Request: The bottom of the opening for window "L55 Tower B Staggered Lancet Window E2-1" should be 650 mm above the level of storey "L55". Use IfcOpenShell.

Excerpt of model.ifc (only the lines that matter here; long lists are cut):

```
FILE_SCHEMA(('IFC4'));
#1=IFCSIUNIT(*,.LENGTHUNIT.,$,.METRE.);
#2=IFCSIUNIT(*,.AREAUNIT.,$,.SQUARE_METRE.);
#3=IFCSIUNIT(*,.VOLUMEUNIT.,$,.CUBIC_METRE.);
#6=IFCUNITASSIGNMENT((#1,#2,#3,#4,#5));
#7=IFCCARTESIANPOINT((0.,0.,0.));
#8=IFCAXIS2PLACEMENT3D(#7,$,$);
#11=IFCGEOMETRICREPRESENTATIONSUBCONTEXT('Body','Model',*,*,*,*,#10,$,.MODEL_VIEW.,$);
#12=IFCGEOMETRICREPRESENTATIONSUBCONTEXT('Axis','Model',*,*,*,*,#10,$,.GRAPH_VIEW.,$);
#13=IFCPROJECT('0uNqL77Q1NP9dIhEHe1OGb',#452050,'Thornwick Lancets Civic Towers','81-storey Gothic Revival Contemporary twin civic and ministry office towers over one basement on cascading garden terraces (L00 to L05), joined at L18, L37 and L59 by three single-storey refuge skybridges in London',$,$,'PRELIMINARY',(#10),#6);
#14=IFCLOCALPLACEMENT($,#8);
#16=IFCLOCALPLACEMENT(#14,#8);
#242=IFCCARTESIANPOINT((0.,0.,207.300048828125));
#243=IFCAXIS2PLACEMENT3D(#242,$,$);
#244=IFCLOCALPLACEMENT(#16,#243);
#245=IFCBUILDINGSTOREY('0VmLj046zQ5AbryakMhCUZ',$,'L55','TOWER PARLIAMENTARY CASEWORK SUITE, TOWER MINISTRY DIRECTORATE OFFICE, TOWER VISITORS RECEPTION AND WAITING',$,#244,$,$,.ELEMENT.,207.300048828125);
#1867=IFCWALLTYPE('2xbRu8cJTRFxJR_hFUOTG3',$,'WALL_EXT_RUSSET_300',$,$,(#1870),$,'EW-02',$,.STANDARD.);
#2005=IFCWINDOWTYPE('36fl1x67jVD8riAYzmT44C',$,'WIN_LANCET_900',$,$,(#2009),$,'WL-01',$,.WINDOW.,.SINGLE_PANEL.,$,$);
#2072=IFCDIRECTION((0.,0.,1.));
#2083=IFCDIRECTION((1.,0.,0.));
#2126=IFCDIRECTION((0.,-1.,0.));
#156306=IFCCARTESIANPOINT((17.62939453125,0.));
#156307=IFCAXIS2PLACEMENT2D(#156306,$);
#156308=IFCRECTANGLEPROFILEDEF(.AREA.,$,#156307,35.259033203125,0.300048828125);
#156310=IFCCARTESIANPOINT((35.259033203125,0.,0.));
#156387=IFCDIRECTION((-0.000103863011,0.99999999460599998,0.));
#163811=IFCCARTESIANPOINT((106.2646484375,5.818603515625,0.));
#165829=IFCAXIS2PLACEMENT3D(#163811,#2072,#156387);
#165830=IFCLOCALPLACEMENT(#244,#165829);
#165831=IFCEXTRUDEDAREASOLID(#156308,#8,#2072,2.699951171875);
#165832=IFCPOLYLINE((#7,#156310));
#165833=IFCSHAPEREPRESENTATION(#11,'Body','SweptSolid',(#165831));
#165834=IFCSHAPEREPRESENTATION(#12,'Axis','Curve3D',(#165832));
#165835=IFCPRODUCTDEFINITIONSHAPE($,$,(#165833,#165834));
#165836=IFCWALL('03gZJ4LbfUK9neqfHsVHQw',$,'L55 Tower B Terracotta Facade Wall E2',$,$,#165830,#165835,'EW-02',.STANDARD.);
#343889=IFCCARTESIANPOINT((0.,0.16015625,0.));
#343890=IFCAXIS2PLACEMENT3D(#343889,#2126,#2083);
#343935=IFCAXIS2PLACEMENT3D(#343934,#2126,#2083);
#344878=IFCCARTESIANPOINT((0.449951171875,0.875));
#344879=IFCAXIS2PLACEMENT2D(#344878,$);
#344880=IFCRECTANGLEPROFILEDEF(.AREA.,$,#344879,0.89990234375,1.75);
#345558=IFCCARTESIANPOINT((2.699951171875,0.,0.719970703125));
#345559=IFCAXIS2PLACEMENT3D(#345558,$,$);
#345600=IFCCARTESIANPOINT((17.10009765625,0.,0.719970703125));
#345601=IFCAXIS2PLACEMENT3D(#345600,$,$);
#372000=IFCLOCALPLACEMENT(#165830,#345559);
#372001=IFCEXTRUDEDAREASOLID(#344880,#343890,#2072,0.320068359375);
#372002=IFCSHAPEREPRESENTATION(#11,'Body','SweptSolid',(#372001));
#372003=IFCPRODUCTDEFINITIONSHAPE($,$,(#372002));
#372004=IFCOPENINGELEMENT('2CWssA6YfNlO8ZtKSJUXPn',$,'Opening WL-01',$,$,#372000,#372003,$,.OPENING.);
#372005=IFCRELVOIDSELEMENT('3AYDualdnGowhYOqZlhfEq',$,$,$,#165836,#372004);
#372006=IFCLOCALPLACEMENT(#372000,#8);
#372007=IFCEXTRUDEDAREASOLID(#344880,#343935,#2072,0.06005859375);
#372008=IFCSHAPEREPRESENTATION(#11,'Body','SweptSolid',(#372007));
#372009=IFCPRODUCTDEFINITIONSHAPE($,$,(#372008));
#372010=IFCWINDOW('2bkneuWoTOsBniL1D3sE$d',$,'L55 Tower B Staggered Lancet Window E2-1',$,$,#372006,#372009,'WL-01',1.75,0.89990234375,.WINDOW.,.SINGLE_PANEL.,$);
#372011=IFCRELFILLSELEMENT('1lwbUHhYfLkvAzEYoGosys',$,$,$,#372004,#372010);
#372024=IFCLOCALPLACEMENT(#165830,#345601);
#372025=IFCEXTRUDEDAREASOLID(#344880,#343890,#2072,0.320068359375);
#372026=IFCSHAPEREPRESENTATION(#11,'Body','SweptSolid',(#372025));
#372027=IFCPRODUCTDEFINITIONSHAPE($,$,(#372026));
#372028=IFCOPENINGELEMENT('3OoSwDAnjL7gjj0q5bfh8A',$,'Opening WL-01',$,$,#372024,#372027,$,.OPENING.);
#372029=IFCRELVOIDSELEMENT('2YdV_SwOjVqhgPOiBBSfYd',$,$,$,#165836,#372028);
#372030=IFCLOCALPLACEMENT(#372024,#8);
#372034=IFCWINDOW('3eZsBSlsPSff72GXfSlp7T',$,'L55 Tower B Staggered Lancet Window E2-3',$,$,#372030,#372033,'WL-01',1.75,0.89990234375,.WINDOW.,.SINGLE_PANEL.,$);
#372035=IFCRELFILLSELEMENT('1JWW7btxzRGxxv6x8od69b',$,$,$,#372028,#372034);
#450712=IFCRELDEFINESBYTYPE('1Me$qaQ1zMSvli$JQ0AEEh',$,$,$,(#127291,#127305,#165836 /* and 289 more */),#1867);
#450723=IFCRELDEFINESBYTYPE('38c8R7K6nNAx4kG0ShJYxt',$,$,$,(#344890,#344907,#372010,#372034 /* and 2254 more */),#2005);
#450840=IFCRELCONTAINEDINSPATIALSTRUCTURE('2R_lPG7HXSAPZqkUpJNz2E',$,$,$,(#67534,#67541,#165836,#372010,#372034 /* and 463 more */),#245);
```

```python
import numpy as np
import ifcopenshell
import ifcopenshell.api.geometry
import ifcopenshell.geom
import ifcopenshell.util.element
import ifcopenshell.util.placement
import ifcopenshell.util.shape
import ifcopenshell.util.unit

model = ifcopenshell.open("model.ifc")
unit_scale = ifcopenshell.util.unit.calculate_unit_scale(model)

window = model.by_guid("2bkneuWoTOsBniL1D3sE$d")
opening = window.FillsVoids[0].RelatingOpeningElement
storey = ifcopenshell.util.element.get_container(window, ifc_class="IfcBuildingStorey")
level = ifcopenshell.util.placement.get_local_placement(storey.ObjectPlacement)[2, 3]

# The opening's origin need not be at the sill, so measure its lowest point.
shape = ifcopenshell.geom.create_shape(ifcopenshell.geom.settings(), opening)
bottom = ifcopenshell.util.shape.get_shape_bottom_elevation(shape, shape.geometry) / unit_scale
dz = level + 0.65 / unit_scale - bottom

shift = np.array([0.0, 0.0, dz])
# The window is placed relative to its opening, so it follows when the opening moves.
matrix = ifcopenshell.util.placement.get_local_placement(opening.ObjectPlacement)
matrix[:3, 3] += shift
ifcopenshell.api.geometry.edit_object_placement(
    model, product=opening, matrix=matrix, is_si=False, should_transform_children=True
)

print(f"moved by {dz * unit_scale:+.3f} m")

model.write("model_v2.ifc")
```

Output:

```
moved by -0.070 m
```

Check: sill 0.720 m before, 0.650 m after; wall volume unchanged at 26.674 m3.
